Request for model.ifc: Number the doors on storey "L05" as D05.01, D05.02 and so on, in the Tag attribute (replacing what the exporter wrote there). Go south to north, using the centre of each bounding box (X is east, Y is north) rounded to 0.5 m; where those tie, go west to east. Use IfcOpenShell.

First a look at what the model holds.

```python
import ifcopenshell
import ifcopenshell.util.element
import ifcopenshell.util.placement

model = ifcopenshell.open("model.ifc")
print(model.schema)
storey = next(s for s in model.by_type("IfcBuildingStorey") if s.Name == "L05")
doors = [e for e in ifcopenshell.util.element.get_decomposition(storey) if e.is_a("IfcDoor")]
for e in sorted(doors, key=lambda e: e.id()):
    origin = ifcopenshell.util.placement.get_local_placement(e.ObjectPlacement)[:3, 3]
    print(e.id(), e.Tag, e.Name, origin.round(2) + 0.0, sep=" | ")
```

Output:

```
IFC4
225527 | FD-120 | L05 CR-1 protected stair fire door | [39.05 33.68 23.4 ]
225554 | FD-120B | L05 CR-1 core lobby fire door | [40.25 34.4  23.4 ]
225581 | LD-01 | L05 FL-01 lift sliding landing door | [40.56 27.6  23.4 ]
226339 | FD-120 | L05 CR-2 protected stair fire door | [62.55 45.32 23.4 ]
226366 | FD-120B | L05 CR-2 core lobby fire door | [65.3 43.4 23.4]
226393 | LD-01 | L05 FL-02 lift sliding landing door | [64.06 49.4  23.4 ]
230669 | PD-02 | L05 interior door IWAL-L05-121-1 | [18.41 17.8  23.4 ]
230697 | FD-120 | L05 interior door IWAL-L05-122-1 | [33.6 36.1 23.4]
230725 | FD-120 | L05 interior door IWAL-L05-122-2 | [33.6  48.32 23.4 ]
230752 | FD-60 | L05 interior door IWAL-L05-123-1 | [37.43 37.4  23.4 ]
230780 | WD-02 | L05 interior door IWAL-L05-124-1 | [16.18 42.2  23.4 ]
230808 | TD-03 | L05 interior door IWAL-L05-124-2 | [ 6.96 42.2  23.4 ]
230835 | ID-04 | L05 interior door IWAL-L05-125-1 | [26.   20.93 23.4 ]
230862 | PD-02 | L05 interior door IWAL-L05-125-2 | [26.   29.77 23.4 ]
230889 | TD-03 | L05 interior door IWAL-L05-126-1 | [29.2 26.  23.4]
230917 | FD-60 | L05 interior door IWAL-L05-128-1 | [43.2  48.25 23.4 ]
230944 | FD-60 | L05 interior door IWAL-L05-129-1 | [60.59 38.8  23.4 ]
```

```python
import ifcopenshell
import ifcopenshell.geom
import ifcopenshell.util.element
import ifcopenshell.util.shape

model = ifcopenshell.open("model.ifc")
settings = ifcopenshell.geom.settings()
settings.set("use-world-coords", True)


def centre(element):
    shape = ifcopenshell.geom.create_shape(settings, element)
    return ifcopenshell.util.shape.get_bbox_centroid(shape.geometry)


storey = next(s for s in model.by_type("IfcBuildingStorey") if s.Name == "L05")
doors = [e for e in ifcopenshell.util.element.get_decomposition(storey) if e.is_a("IfcDoor")]

# Insertion points can sit at a corner or the storey origin, so sort by the geometry (in metres).
centres = {e: centre(e) for e in doors}
doors.sort(key=lambda e: (round(centres[e][1] / 0.5), centres[e][0]))

for i, e in enumerate(doors, start=1):
    number = f"D05.{i:02d}"
    e.Tag = number
    print(e.id(), number)

model.write("model_updated.ifc")
```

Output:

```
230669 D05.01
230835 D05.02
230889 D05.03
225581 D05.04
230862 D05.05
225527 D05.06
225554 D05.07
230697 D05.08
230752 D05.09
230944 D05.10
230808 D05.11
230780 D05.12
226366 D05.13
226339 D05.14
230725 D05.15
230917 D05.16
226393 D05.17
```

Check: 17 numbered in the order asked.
